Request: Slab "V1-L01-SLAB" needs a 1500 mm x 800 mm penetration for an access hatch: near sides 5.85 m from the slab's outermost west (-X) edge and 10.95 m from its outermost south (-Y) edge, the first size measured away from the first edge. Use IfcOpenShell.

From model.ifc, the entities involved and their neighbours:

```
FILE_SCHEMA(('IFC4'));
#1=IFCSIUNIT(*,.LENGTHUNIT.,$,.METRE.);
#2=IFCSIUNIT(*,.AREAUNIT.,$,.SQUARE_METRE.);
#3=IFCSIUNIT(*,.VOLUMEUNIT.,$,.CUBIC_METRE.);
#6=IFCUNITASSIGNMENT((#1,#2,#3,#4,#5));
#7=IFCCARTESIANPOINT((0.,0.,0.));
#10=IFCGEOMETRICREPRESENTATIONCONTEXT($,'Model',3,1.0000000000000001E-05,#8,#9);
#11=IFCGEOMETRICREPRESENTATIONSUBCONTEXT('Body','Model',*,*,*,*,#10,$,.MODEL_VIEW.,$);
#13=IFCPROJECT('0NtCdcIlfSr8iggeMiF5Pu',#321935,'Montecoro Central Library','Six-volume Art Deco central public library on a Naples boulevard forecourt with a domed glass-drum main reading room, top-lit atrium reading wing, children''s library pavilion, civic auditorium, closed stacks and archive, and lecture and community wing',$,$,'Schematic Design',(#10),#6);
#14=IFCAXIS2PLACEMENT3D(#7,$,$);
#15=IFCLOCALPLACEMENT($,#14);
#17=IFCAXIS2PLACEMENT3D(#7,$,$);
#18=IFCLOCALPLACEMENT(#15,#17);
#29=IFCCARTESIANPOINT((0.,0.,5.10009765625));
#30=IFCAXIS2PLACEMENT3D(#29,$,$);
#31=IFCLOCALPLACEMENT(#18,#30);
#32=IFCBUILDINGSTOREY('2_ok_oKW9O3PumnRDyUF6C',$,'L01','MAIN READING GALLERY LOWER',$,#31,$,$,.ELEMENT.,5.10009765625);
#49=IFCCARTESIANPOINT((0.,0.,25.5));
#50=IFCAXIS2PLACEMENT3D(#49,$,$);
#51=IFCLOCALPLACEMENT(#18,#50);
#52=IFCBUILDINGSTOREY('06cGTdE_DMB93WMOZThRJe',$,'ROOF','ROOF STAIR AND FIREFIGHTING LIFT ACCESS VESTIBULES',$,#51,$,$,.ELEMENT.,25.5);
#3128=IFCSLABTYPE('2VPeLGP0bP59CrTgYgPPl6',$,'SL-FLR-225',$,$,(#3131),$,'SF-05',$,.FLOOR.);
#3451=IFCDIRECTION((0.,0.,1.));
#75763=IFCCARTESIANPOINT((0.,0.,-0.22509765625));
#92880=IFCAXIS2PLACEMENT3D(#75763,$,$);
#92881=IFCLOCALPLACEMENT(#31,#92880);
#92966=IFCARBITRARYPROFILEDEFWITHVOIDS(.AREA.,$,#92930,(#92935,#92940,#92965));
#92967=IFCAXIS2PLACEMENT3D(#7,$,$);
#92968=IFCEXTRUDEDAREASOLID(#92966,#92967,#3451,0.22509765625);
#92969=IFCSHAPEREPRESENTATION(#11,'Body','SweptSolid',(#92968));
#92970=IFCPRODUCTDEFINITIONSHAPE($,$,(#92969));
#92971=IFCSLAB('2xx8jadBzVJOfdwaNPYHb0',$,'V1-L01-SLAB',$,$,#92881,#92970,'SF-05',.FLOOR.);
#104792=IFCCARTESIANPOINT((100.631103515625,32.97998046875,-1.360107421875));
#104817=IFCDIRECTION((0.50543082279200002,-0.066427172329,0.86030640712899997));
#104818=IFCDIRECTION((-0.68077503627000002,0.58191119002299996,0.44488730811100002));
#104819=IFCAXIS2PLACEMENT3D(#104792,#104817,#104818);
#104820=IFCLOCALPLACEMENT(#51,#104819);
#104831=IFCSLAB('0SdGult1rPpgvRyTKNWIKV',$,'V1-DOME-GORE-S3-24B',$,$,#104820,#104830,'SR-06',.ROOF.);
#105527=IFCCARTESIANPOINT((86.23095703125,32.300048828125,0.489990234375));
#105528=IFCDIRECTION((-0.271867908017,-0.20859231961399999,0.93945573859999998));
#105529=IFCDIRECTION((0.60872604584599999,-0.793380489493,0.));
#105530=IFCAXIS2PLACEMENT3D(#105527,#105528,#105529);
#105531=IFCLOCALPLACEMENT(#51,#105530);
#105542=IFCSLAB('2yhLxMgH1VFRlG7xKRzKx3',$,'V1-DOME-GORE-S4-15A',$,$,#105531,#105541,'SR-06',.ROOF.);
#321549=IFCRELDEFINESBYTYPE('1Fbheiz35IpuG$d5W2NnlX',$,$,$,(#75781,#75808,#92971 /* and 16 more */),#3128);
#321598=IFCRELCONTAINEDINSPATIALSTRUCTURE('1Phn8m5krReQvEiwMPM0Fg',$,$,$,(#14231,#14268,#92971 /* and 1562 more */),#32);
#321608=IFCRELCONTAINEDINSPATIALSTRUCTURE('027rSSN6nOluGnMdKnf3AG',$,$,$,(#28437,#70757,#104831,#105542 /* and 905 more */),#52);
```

```python
import numpy as np
import ifcopenshell
import ifcopenshell.api.feature
import ifcopenshell.api.geometry
import ifcopenshell.api.root
import ifcopenshell.geom
import ifcopenshell.util.placement
import ifcopenshell.util.representation
import ifcopenshell.util.shape
import ifcopenshell.util.unit

model = ifcopenshell.open("model.ifc")
unit_scale = ifcopenshell.util.unit.calculate_unit_scale(model)
settings = ifcopenshell.geom.settings()


def volume(element):
    """Net volume in cubic metres, openings subtracted."""
    shape = ifcopenshell.geom.create_shape(settings, element)
    return ifcopenshell.util.shape.get_volume(shape.geometry)


slab = model.by_guid("2xx8jadBzVJOfdwaNPYHb0")
before = volume(slab)

# Extent in the slab's own axes, in metres. The edges named are its -X and -Y sides.
slab_shape = ifcopenshell.geom.create_shape(settings, slab)
vertices = ifcopenshell.util.shape.get_vertices(slab_shape.geometry)
x_min, y_min, bottom = vertices.min(axis=0)
top = vertices[:, 2].max()

opening = ifcopenshell.api.root.create_entity(model, ifc_class="IfcOpeningElement", name="Access hatch opening", predefined_type="OPENING")
context = ifcopenshell.util.representation.get_context(model, "Model", "Body", "MODEL_VIEW")
width, depth = 1.5, 0.8
outline = [(0.0, 0.0), (width, 0.0), (width, depth), (0.0, depth), (0.0, 0.0)]
# Overshoot both faces by 50 mm so the cut is clean.
shape = ifcopenshell.api.geometry.add_slab_representation(
    model, context=context, depth=top - bottom + 0.1, polyline=outline
)
ifcopenshell.api.geometry.assign_representation(model, product=opening, representation=shape)

matrix = ifcopenshell.util.placement.get_local_placement(slab.ObjectPlacement)
matrix[:, 3] = matrix @ np.append(np.array([x_min + 5.85, y_min + 10.95, bottom - 0.05]) / unit_scale, 1.0)
ifcopenshell.api.geometry.edit_object_placement(model, product=opening, matrix=matrix, is_si=False)
ifcopenshell.api.feature.add_feature(model, feature=opening, element=slab)

after = volume(slab)

print(f"slab volume {before:.3f} -> {after:.3f} m3")

model.write("model_rev.ifc")
```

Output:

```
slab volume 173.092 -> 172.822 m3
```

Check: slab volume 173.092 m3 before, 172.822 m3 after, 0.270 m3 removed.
